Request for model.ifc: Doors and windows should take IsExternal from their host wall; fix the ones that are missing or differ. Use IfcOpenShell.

First a look at what the model holds.

```python
import ifcopenshell
import ifcopenshell.util.element

model = ifcopenshell.open("model.ifc")
print(model.schema)
seen = {}
for e in model.by_type("IfcDoor") + model.by_type("IfcWindow"):
    if not e.FillsVoids:
        continue
    host = e.FillsVoids[0].RelatingOpeningElement.VoidsElements[0].RelatingBuildingElement
    own = ifcopenshell.util.element.get_pset(e, f"Pset_{e.is_a()[3:].removesuffix('StandardCase')}Common", "IsExternal")
    wall = ifcopenshell.util.element.get_pset(host, "Pset_WallCommon", "IsExternal")
    seen[e.is_a(), own, wall] = seen.get((e.is_a(), own, wall), 0) + 1
for (cls, own, wall), count in sorted(seen.items(), key=str):
    print(count, cls, "IsExternal:", own, "| host wall:", wall)
```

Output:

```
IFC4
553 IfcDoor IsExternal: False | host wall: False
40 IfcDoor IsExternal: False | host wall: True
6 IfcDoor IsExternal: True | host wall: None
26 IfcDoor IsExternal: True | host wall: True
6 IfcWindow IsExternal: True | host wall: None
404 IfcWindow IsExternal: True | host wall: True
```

```python
import ifcopenshell
import ifcopenshell.api.pset
import ifcopenshell.util.element

model = ifcopenshell.open("model.ifc")

count = 0
for ifc_class, pset_name in (("IfcDoor", "Pset_DoorCommon"), ("IfcWindow", "Pset_WindowCommon")):
    for e in model.by_type(ifc_class):
        if not e.FillsVoids:
            continue
        host = e.FillsVoids[0].RelatingOpeningElement.VoidsElements[0].RelatingBuildingElement
        external = ifcopenshell.util.element.get_pset(host, "Pset_WallCommon", "IsExternal")
        if external is None or ifcopenshell.util.element.get_pset(e, pset_name, "IsExternal") == external:
            continue
        pset = ifcopenshell.api.pset.add_pset(model, product=e, name=pset_name)
        ifcopenshell.api.pset.edit_pset(model, pset=pset, properties={"IsExternal": external})
        count += 1

print(count, "updated")

model.write("model_edited.ifc")
```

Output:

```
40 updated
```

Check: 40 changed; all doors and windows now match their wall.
